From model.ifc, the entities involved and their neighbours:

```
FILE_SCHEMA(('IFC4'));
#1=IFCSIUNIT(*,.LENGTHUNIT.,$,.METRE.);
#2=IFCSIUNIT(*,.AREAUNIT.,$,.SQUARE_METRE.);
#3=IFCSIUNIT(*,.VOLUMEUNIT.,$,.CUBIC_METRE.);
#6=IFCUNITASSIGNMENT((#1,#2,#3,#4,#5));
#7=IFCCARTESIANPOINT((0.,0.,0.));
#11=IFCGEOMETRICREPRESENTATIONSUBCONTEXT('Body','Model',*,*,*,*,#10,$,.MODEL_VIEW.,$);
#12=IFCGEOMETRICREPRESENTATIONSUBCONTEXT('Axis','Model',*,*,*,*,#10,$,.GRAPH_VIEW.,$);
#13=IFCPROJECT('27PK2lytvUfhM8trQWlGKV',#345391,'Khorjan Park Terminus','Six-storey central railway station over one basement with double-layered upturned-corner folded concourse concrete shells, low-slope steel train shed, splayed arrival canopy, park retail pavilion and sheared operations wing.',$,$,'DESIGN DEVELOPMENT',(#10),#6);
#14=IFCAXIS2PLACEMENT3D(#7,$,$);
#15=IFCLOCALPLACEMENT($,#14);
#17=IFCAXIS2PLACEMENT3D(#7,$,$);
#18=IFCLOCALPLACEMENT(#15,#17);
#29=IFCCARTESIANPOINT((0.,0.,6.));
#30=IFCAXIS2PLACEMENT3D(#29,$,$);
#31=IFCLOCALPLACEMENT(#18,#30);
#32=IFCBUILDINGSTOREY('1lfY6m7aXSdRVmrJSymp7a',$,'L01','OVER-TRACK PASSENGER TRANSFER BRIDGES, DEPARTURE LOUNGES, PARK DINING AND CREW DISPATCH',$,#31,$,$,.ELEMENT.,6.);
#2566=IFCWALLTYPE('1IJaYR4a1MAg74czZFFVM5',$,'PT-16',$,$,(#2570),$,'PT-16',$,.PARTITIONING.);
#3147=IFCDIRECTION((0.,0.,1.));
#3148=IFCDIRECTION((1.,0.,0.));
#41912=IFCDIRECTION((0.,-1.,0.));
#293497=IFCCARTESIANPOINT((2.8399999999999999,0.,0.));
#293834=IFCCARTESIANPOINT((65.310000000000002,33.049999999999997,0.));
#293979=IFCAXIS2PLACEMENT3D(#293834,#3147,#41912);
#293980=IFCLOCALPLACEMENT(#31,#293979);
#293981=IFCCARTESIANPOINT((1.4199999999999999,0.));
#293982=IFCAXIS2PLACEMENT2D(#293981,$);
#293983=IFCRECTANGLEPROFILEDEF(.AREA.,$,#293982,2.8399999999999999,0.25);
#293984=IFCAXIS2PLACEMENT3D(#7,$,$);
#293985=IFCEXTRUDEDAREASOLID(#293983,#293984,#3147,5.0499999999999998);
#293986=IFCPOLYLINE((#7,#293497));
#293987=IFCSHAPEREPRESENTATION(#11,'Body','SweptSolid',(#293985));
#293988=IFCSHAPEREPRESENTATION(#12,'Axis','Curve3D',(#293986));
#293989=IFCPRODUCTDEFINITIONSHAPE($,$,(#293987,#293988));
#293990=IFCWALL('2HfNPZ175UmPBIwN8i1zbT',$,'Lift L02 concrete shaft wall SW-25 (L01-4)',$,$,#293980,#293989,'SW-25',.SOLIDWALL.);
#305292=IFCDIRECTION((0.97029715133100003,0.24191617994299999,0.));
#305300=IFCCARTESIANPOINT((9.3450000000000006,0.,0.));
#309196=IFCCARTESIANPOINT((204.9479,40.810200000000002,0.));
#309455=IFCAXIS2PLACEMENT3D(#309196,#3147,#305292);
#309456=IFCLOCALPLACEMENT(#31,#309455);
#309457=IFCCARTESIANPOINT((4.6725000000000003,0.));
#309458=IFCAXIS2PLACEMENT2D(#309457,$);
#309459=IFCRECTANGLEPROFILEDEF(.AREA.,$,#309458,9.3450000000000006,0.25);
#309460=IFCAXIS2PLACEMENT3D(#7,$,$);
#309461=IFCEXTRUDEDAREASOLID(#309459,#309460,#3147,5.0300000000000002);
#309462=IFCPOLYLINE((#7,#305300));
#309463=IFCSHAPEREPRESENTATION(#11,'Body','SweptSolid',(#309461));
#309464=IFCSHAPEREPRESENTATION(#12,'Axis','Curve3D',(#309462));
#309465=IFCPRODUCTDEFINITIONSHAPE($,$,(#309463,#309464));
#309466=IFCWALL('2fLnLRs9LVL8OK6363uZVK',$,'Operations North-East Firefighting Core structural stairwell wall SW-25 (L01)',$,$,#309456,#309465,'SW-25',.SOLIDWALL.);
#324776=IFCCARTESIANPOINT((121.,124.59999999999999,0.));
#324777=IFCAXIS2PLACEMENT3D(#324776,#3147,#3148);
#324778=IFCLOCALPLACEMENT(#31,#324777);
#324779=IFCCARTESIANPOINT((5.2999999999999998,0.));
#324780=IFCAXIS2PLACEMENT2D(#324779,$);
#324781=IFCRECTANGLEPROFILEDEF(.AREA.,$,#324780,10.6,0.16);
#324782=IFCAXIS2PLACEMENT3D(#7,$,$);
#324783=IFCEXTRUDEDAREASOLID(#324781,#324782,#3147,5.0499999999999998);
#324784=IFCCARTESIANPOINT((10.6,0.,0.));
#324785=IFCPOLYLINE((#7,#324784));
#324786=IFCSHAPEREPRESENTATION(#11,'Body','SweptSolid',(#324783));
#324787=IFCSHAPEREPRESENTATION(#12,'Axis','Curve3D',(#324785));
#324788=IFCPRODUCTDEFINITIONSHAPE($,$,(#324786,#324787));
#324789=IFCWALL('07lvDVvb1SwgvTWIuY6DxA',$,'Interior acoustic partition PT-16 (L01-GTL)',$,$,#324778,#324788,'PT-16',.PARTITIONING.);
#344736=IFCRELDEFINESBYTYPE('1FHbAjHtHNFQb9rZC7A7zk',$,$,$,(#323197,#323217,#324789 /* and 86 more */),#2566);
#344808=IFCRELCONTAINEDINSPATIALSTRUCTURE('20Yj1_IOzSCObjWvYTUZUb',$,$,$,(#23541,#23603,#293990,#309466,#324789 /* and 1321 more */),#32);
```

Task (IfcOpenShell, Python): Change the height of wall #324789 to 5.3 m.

```python
import ifcopenshell
import ifcopenshell.geom
import ifcopenshell.util.representation
import ifcopenshell.util.shape

model = ifcopenshell.open("model.ifc")
settings = ifcopenshell.geom.settings()


def volume(element):
    """Net volume in cubic metres, openings subtracted."""
    shape = ifcopenshell.geom.create_shape(settings, element)
    return ifcopenshell.util.shape.get_volume(shape.geometry)


wall = model.by_guid("07lvDVvb1SwgvTWIuY6DxA")
before = volume(wall)

body = ifcopenshell.util.representation.get_representation(wall, "Model", "Body")
solid = body.Items[0]
old_height = solid.Depth
solid.Depth = 5.3
after = volume(wall)

print(f"height {old_height:g} -> {solid.Depth:g}, volume {before:.3f} -> {after:.3f} m3")

model.write("model_rev.ifc")
```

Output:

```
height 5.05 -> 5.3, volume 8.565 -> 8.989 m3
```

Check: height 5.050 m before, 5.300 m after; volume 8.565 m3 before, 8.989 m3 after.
